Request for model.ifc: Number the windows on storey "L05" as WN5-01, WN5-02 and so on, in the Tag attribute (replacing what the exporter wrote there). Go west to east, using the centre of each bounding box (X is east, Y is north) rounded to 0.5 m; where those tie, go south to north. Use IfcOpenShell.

First a look at what the model holds.

```python
import ifcopenshell
import ifcopenshell.util.element
import ifcopenshell.util.placement

model = ifcopenshell.open("model.ifc")
print(model.schema)
storey = next(s for s in model.by_type("IfcBuildingStorey") if s.Name == "L05")
windows = [e for e in ifcopenshell.util.element.get_decomposition(storey) if e.is_a("IfcWindow")]
for e in sorted(windows, key=lambda e: e.id()):
    origin = ifcopenshell.util.placement.get_local_placement(e.ObjectPlacement)[:3, 3]
    print(e.id(), e.Tag, e.Name, origin.round(2) + 0.0, sep=" | ")
```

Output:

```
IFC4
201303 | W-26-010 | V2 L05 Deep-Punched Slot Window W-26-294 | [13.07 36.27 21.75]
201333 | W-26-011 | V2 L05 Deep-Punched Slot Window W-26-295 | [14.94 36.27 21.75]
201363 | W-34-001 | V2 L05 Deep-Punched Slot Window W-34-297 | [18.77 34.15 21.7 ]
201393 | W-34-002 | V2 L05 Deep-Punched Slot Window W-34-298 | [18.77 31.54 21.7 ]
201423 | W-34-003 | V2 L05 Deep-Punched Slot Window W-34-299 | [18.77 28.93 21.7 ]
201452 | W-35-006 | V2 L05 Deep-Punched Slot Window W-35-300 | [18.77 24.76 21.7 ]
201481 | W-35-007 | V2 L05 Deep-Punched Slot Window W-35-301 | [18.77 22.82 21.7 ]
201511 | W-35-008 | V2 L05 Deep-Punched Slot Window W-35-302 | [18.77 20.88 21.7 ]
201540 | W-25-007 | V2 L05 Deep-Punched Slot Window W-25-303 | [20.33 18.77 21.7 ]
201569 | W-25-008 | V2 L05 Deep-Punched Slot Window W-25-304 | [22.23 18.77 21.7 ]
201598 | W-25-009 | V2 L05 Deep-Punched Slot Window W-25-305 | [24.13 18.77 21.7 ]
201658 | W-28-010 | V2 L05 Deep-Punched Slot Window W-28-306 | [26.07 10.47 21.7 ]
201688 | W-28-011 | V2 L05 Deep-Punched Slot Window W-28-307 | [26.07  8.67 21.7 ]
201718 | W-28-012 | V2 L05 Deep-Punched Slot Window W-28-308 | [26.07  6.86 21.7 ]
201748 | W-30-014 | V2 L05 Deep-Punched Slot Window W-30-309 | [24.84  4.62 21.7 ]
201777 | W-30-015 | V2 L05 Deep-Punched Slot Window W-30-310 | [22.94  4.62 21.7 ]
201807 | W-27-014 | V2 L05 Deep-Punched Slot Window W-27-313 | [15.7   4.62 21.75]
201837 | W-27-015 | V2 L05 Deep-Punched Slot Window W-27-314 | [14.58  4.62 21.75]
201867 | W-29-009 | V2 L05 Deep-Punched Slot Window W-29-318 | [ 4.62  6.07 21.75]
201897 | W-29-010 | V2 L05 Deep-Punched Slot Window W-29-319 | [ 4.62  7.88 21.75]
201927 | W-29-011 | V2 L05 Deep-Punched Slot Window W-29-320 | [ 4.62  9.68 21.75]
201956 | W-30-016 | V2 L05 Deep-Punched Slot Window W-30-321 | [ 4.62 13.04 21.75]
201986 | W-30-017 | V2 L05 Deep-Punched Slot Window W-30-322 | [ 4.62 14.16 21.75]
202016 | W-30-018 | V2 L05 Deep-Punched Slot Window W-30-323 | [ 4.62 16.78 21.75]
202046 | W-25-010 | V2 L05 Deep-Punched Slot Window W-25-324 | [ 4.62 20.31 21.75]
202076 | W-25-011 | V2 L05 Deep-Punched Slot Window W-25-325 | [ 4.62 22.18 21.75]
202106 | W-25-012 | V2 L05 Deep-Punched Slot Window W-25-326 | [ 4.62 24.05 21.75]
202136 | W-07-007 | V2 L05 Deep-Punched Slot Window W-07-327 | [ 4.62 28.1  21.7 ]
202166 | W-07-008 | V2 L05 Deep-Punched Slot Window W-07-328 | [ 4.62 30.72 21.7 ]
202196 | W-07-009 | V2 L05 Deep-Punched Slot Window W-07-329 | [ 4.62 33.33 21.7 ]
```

```python
import ifcopenshell
import ifcopenshell.geom
import ifcopenshell.util.element
import ifcopenshell.util.shape

model = ifcopenshell.open("model.ifc")
settings = ifcopenshell.geom.settings()
settings.set("use-world-coords", True)


def centre(element):
    shape = ifcopenshell.geom.create_shape(settings, element)
    return ifcopenshell.util.shape.get_bbox_centroid(shape.geometry)


storey = next(s for s in model.by_type("IfcBuildingStorey") if s.Name == "L05")
windows = [e for e in ifcopenshell.util.element.get_decomposition(storey) if e.is_a("IfcWindow")]

# Insertion points can sit at a corner or the storey origin, so sort by the geometry (in metres).
centres = {e: centre(e) for e in windows}
windows.sort(key=lambda e: (round(centres[e][0] / 0.5), centres[e][1]))

for i, e in enumerate(windows, start=1):
    number = f"WN5-{i:02d}"
    e.Tag = number
    print(e.id(), number)

model.write("model-out.ifc")
```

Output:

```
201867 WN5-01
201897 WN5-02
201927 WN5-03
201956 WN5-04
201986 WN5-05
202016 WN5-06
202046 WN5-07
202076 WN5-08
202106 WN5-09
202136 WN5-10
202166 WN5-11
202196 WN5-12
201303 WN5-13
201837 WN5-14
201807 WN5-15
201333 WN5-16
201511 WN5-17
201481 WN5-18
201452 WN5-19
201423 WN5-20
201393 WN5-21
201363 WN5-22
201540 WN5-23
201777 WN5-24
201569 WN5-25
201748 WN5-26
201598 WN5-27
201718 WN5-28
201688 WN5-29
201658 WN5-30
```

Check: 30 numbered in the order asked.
